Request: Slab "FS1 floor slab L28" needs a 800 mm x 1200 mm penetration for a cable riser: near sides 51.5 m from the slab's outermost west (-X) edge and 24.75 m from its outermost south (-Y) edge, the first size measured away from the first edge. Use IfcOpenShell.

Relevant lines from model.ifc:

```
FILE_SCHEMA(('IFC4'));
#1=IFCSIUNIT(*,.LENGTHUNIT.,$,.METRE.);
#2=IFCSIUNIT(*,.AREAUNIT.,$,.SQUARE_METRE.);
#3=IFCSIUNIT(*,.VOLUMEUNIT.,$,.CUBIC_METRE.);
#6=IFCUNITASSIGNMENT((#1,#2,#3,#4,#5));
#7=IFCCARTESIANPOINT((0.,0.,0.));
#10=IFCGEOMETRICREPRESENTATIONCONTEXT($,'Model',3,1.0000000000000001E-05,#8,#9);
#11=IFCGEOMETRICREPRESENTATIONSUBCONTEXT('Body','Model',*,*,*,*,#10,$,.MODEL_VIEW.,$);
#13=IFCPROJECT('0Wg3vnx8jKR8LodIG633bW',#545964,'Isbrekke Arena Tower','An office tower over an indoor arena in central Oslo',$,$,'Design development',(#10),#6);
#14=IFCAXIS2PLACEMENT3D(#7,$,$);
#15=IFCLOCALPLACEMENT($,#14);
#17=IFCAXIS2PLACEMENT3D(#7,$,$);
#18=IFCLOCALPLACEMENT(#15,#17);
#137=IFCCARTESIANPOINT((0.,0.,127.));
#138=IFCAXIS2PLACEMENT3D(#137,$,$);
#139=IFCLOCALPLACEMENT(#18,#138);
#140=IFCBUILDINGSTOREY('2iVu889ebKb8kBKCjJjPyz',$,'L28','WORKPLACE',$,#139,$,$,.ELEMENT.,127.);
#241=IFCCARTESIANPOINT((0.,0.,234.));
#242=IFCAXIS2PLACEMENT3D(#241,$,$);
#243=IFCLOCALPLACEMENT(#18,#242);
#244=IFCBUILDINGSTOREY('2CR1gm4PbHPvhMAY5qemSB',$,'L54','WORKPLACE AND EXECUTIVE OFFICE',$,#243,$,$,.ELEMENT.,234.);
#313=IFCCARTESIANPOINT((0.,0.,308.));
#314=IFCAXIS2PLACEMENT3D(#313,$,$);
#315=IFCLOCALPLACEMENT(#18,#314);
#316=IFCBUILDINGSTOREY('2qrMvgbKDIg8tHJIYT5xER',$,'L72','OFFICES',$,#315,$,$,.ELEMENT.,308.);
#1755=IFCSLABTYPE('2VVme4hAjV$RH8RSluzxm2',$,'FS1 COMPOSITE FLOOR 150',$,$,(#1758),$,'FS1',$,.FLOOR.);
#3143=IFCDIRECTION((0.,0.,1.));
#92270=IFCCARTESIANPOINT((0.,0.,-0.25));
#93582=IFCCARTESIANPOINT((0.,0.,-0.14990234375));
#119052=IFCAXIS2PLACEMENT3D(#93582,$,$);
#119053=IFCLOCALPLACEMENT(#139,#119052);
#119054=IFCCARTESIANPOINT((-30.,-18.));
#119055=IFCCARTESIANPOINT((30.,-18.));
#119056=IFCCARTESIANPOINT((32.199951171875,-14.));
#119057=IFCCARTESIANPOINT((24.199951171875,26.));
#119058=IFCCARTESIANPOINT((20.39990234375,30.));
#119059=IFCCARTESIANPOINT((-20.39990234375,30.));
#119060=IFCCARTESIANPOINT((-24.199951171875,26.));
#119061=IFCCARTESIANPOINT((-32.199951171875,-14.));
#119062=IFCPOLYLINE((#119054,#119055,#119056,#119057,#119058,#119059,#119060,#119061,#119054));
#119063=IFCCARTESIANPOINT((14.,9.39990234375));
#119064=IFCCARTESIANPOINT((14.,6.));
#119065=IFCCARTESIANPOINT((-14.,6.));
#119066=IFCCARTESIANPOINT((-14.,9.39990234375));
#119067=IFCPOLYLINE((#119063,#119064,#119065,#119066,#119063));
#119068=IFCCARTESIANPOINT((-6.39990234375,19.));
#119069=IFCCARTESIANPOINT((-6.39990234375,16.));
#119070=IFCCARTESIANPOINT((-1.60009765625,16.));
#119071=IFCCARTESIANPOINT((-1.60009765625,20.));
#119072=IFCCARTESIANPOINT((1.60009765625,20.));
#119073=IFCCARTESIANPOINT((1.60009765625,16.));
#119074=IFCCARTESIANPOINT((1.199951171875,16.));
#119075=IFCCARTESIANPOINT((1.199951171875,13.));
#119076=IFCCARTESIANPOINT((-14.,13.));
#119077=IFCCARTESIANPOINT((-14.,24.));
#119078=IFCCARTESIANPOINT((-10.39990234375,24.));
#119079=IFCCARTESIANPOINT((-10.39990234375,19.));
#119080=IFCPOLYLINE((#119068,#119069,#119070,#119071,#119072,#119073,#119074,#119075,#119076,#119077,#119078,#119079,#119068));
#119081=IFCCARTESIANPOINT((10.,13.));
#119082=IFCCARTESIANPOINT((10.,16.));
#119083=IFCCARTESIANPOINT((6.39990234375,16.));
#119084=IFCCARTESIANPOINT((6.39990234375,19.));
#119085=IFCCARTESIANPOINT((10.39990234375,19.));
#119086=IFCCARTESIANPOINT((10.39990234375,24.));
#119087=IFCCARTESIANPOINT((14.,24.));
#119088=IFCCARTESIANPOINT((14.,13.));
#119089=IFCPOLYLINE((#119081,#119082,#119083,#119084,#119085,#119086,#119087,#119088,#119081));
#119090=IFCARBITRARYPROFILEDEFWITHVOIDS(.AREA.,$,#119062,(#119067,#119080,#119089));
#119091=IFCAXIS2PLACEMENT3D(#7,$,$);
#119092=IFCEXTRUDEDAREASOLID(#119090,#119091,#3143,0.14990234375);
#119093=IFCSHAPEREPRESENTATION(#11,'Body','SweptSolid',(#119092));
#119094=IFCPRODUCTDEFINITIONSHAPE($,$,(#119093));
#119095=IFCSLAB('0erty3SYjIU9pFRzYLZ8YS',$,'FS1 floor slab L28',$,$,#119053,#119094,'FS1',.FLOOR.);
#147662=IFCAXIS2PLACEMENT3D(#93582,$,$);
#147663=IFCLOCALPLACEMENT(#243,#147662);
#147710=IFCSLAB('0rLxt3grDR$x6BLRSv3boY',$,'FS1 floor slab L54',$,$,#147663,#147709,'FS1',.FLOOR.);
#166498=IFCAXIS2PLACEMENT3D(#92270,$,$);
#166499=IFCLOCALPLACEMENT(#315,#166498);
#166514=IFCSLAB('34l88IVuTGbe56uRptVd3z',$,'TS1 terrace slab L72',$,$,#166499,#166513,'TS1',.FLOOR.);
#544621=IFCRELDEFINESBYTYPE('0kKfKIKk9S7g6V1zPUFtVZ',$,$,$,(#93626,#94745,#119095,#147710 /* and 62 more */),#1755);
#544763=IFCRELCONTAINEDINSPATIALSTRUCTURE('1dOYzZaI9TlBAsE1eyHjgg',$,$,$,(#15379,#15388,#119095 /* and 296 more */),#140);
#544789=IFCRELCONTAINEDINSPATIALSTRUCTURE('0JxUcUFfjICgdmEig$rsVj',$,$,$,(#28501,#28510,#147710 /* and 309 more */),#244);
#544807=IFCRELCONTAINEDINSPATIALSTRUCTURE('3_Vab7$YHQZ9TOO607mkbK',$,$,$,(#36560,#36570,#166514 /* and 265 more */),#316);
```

```python
import numpy as np
import ifcopenshell
import ifcopenshell.api.feature
import ifcopenshell.api.geometry
import ifcopenshell.api.root
import ifcopenshell.geom
import ifcopenshell.util.placement
import ifcopenshell.util.representation
import ifcopenshell.util.shape
import ifcopenshell.util.unit

model = ifcopenshell.open("model.ifc")
unit_scale = ifcopenshell.util.unit.calculate_unit_scale(model)
settings = ifcopenshell.geom.settings()


def volume(element):
    """Net volume in cubic metres, openings subtracted."""
    shape = ifcopenshell.geom.create_shape(settings, element)
    return ifcopenshell.util.shape.get_volume(shape.geometry)


slab = model.by_id(119095)
before = volume(slab)

# Extent in the slab's own axes, in metres. The edges named are its -X and -Y sides.
slab_shape = ifcopenshell.geom.create_shape(settings, slab)
vertices = ifcopenshell.util.shape.get_vertices(slab_shape.geometry)
x_min, y_min, bottom = vertices.min(axis=0)
top = vertices[:, 2].max()

opening = ifcopenshell.api.root.create_entity(model, ifc_class="IfcOpeningElement", name="Cable riser opening", predefined_type="OPENING")
context = ifcopenshell.util.representation.get_context(model, "Model", "Body", "MODEL_VIEW")
width, depth = 0.8, 1.2
outline = [(0.0, 0.0), (width, 0.0), (width, depth), (0.0, depth), (0.0, 0.0)]
# Overshoot both faces by 50 mm so the cut is clean.
shape = ifcopenshell.api.geometry.add_slab_representation(
    model, context=context, depth=top - bottom + 0.1, polyline=outline
)
ifcopenshell.api.geometry.assign_representation(model, product=opening, representation=shape)

matrix = ifcopenshell.util.placement.get_local_placement(slab.ObjectPlacement)
matrix[:, 3] = matrix @ np.append(np.array([x_min + 51.5, y_min + 24.75, bottom - 0.05]) / unit_scale, 1.0)
ifcopenshell.api.geometry.edit_object_placement(model, product=opening, matrix=matrix, is_si=False)
ifcopenshell.api.feature.add_feature(model, feature=opening, element=slab)

after = volume(slab)

print(f"slab volume {before:.3f} -> {after:.3f} m3")

model.write("model_updated.ifc")
```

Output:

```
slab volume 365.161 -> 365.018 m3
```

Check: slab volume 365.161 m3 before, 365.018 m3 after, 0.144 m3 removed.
